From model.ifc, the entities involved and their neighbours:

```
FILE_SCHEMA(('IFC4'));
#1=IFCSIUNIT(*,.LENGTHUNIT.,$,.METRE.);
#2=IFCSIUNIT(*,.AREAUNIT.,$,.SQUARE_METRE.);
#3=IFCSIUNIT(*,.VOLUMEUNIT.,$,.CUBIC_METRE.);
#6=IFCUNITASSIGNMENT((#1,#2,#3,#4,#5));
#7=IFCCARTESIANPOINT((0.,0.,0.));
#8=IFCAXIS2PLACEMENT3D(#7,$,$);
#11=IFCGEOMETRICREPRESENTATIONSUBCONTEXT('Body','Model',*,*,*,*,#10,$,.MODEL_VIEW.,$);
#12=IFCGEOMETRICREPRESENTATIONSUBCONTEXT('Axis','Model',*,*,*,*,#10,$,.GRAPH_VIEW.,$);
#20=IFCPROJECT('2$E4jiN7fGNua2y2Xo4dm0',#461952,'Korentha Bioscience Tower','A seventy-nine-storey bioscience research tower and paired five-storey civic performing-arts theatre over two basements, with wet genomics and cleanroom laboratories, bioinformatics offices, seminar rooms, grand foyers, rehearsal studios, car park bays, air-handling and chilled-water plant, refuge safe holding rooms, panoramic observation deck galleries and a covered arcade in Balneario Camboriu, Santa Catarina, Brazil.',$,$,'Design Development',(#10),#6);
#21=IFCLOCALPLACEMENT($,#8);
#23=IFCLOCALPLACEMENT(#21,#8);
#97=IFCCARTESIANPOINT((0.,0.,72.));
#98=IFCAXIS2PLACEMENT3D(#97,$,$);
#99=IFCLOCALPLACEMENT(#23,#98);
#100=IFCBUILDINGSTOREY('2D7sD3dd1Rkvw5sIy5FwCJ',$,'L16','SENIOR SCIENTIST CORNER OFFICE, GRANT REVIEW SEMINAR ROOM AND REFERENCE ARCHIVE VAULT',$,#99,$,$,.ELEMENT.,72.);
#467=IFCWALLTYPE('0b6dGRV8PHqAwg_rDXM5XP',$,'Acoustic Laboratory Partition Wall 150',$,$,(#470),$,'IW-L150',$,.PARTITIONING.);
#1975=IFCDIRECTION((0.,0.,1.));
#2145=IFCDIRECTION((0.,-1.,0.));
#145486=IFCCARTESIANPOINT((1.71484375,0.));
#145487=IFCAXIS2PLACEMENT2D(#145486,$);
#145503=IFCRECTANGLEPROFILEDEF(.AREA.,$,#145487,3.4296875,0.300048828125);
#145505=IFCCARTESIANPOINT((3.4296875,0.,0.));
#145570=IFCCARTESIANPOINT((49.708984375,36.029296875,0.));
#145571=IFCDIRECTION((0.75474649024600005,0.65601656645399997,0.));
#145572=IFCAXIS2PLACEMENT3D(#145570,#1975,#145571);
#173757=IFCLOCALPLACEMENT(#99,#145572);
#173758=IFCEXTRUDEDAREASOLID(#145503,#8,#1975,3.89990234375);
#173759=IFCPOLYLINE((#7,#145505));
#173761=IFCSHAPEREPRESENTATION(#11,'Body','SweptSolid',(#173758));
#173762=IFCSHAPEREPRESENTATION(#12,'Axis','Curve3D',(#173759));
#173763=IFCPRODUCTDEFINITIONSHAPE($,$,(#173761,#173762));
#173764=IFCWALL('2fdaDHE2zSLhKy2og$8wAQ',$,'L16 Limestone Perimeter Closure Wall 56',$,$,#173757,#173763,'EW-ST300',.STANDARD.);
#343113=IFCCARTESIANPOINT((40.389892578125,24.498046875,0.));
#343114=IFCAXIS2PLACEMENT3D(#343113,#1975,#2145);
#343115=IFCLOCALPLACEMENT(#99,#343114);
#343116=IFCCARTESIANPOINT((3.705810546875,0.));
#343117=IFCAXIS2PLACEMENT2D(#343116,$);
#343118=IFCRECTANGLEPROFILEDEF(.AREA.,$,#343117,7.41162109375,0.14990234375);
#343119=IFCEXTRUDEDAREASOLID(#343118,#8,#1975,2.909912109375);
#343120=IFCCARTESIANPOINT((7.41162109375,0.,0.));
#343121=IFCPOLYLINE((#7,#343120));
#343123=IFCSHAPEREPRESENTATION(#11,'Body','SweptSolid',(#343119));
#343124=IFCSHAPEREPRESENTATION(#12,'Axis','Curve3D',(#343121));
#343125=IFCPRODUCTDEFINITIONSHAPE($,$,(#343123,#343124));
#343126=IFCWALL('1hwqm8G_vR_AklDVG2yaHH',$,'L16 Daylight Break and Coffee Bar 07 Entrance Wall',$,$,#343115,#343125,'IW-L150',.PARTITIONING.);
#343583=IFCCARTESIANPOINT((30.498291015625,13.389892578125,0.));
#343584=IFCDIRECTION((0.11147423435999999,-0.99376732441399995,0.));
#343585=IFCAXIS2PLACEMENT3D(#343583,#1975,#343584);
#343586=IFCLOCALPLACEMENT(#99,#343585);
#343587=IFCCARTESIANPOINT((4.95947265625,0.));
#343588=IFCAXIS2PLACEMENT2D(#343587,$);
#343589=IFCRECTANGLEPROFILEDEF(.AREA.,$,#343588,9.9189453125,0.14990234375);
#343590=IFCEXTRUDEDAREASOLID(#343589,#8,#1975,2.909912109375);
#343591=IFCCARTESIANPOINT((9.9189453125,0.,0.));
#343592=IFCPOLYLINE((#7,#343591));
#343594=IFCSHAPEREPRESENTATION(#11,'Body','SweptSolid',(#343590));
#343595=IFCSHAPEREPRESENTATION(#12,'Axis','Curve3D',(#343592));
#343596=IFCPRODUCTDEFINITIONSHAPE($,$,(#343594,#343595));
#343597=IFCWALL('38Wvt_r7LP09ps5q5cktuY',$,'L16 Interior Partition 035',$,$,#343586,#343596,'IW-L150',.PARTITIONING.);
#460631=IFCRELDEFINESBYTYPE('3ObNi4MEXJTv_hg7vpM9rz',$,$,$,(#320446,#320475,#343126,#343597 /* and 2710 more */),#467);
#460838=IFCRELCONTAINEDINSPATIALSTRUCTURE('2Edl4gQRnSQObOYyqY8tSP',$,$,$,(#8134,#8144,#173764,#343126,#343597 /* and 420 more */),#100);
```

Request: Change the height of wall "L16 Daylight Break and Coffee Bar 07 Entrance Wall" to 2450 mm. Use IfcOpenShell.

```python
import ifcopenshell
import ifcopenshell.geom
import ifcopenshell.util.representation
import ifcopenshell.util.shape
import ifcopenshell.util.unit

model = ifcopenshell.open("model.ifc")
unit_scale = ifcopenshell.util.unit.calculate_unit_scale(model)
settings = ifcopenshell.geom.settings()


def volume(element):
    """Net volume in cubic metres, openings subtracted."""
    shape = ifcopenshell.geom.create_shape(settings, element)
    return ifcopenshell.util.shape.get_volume(shape.geometry)


wall = model.by_guid("1hwqm8G_vR_AklDVG2yaHH")
before = volume(wall)

body = ifcopenshell.util.representation.get_representation(wall, "Model", "Body")
solid = body.Items[0]
old_height = solid.Depth
solid.Depth = 2.45 / unit_scale
after = volume(wall)

print(f"height {old_height:g} -> {solid.Depth:g}, volume {before:.3f} -> {after:.3f} m3")

model.write("model_rev.ifc")
```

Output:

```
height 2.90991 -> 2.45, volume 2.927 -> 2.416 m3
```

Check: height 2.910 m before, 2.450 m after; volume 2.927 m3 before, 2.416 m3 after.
